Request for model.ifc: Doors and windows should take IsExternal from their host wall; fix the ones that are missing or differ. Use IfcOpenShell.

First a look at what the model holds.

```python
import ifcopenshell
import ifcopenshell.util.element

model = ifcopenshell.open("model.ifc")
print(model.schema)
seen = {}
for e in model.by_type("IfcDoor") + model.by_type("IfcWindow"):
    if not e.FillsVoids:
        continue
    host = e.FillsVoids[0].RelatingOpeningElement.VoidsElements[0].RelatingBuildingElement
    own = ifcopenshell.util.element.get_pset(e, f"Pset_{e.is_a()[3:].removesuffix('StandardCase')}Common", "IsExternal")
    wall = ifcopenshell.util.element.get_pset(host, "Pset_WallCommon", "IsExternal")
    seen[e.is_a(), own, wall] = seen.get((e.is_a(), own, wall), 0) + 1
for (cls, own, wall), count in sorted(seen.items(), key=str):
    print(count, cls, "IsExternal:", own, "| host wall:", wall)
```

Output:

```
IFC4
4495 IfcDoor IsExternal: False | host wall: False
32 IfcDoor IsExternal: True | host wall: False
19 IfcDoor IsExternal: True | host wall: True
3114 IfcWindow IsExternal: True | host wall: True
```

```python
import ifcopenshell
import ifcopenshell.api.pset
import ifcopenshell.util.element

model = ifcopenshell.open("model.ifc")

count = 0
for ifc_class, pset_name in (("IfcDoor", "Pset_DoorCommon"), ("IfcWindow", "Pset_WindowCommon")):
    for e in model.by_type(ifc_class):
        if not e.FillsVoids:
            continue
        host = e.FillsVoids[0].RelatingOpeningElement.VoidsElements[0].RelatingBuildingElement
        external = ifcopenshell.util.element.get_pset(host, "Pset_WallCommon", "IsExternal")
        if external is None or ifcopenshell.util.element.get_pset(e, pset_name, "IsExternal") == external:
            continue
        pset = ifcopenshell.api.pset.add_pset(model, product=e, name=pset_name)
        ifcopenshell.api.pset.edit_pset(model, pset=pset, properties={"IsExternal": external})
        count += 1

print(count, "updated")

model.write("model_rev.ifc")
```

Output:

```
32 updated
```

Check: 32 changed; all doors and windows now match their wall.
